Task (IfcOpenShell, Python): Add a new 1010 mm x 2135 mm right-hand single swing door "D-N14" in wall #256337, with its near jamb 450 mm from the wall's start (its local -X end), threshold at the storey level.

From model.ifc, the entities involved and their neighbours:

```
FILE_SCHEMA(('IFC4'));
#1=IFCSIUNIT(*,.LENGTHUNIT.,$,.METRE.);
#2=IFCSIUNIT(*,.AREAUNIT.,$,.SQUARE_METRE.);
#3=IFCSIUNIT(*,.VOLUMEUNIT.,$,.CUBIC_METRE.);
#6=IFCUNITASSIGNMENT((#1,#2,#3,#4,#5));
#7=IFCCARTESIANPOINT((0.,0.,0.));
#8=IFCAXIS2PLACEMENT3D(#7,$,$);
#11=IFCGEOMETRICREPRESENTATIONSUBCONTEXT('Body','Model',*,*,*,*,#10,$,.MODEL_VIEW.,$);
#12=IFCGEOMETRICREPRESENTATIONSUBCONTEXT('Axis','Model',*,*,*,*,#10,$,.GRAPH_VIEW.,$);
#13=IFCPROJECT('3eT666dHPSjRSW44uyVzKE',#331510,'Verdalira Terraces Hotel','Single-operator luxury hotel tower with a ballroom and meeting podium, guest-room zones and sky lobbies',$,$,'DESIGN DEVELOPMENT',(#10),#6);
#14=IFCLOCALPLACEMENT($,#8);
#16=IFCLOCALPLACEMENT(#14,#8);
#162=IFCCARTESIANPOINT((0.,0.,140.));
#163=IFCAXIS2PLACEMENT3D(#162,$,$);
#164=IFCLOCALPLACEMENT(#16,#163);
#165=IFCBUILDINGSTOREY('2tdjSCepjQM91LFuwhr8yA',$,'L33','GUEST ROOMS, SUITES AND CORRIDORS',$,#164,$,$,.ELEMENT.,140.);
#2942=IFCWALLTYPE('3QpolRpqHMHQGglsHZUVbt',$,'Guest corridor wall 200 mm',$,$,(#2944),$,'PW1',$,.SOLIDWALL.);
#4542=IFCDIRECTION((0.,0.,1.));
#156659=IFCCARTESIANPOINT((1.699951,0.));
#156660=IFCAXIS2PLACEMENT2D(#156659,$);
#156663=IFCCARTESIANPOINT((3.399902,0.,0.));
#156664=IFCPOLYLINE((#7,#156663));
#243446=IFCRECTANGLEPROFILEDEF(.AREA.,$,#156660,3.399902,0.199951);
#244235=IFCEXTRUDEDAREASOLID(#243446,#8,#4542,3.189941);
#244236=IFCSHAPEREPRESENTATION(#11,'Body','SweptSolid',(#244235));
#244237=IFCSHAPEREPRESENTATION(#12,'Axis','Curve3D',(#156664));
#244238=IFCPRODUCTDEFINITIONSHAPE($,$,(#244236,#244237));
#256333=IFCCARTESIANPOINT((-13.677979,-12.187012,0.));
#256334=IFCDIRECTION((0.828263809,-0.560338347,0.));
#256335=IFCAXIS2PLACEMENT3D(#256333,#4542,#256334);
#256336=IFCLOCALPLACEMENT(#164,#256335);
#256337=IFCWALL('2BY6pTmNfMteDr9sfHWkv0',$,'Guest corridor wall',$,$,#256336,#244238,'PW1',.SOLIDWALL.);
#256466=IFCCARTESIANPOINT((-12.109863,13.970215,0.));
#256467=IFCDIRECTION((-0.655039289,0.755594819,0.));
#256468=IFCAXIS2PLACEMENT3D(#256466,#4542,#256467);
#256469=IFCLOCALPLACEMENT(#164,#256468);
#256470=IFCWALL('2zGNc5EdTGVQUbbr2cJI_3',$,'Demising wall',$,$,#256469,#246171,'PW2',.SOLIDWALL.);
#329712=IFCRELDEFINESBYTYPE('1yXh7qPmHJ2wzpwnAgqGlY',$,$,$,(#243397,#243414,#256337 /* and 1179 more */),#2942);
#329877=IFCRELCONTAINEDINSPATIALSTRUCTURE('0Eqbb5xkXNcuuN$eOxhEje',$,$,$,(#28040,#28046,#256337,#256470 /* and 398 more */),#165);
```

```python
import numpy as np
import ifcopenshell
import ifcopenshell.api.feature
import ifcopenshell.api.geometry
import ifcopenshell.api.root
import ifcopenshell.api.spatial
import ifcopenshell.geom
import ifcopenshell.util.element
import ifcopenshell.util.placement
import ifcopenshell.util.representation
import ifcopenshell.util.shape
import ifcopenshell.util.unit

model = ifcopenshell.open("model.ifc")
unit_scale = ifcopenshell.util.unit.calculate_unit_scale(model)
settings = ifcopenshell.geom.settings()


def volume(element):
    """Net volume in cubic metres, openings subtracted."""
    shape = ifcopenshell.geom.create_shape(settings, element)
    return ifcopenshell.util.shape.get_volume(shape.geometry)


wall = model.by_guid("2BY6pTmNfMteDr9sfHWkv0")
storey = ifcopenshell.util.element.get_container(wall, ifc_class="IfcBuildingStorey")
context = ifcopenshell.util.representation.get_context(model, "Model", "Body", "MODEL_VIEW")
before = volume(wall)

width, height, from_end, sill = 1.01, 2.135, 0.45, 0.0  # metres

# The wall runs along its own X axis, and the end named is its -X end.
wall_shape = ifcopenshell.geom.create_shape(settings, wall)
x, y, z = ifcopenshell.util.shape.get_vertices(wall_shape.geometry).T
start = x.min() + from_end
face, thickness = float(y.min()), float(y.max() - y.min())
wall_matrix = ifcopenshell.util.placement.get_local_placement(wall.ObjectPlacement)
level = ifcopenshell.util.placement.get_local_placement(storey.ObjectPlacement)[2, 3]


def in_wall(x, y):
    """Placement at x, y metres in the wall's axes, at sill height."""
    matrix = wall_matrix.copy()
    matrix[:, 3] = wall_matrix @ np.array([x / unit_scale, y / unit_scale, 0.0, 1.0])
    matrix[2, 3] = level + sill / unit_scale
    return matrix


# Opening: a box that overshoots both wall faces by 50 mm.
opening = ifcopenshell.api.root.create_entity(model, ifc_class="IfcOpeningElement", predefined_type="OPENING")
box = ifcopenshell.api.geometry.add_wall_representation(
    model, context=context, length=width, height=height, thickness=thickness + 0.1
)
ifcopenshell.api.geometry.assign_representation(model, product=opening, representation=box)
ifcopenshell.api.geometry.edit_object_placement(model, product=opening, matrix=in_wall(start, face - 0.05), is_si=False)
ifcopenshell.api.feature.add_feature(model, feature=opening, element=wall)

door = ifcopenshell.api.root.create_entity(model, ifc_class="IfcDoor", name="D-N14", predefined_type="DOOR")
door.OverallWidth, door.OverallHeight = width / unit_scale, height / unit_scale
door.OperationType = "SINGLE_SWING_RIGHT"
body = ifcopenshell.api.geometry.add_door_representation(
    model,
    context=context,
    overall_width=door.OverallWidth,
    overall_height=door.OverallHeight,
    operation_type="SINGLE_SWING_RIGHT",
    lining_properties={"LiningDepth": thickness / unit_scale, "ThresholdDepth": thickness / unit_scale},
)
ifcopenshell.api.geometry.assign_representation(model, product=door, representation=body)
ifcopenshell.api.spatial.assign_container(model, products=[door], relating_structure=storey)
ifcopenshell.api.feature.add_filling(model, opening=opening, element=door)

# The lining spans the wall, so the door starts at the wall face.
ifcopenshell.api.geometry.edit_object_placement(model, product=door, matrix=in_wall(start, face), is_si=False)

after = volume(wall)

print(f"wall volume {before:.3f} -> {after:.3f} m3")

model.write("model_edited.ifc")
```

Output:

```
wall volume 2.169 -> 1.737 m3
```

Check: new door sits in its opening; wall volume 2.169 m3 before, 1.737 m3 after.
